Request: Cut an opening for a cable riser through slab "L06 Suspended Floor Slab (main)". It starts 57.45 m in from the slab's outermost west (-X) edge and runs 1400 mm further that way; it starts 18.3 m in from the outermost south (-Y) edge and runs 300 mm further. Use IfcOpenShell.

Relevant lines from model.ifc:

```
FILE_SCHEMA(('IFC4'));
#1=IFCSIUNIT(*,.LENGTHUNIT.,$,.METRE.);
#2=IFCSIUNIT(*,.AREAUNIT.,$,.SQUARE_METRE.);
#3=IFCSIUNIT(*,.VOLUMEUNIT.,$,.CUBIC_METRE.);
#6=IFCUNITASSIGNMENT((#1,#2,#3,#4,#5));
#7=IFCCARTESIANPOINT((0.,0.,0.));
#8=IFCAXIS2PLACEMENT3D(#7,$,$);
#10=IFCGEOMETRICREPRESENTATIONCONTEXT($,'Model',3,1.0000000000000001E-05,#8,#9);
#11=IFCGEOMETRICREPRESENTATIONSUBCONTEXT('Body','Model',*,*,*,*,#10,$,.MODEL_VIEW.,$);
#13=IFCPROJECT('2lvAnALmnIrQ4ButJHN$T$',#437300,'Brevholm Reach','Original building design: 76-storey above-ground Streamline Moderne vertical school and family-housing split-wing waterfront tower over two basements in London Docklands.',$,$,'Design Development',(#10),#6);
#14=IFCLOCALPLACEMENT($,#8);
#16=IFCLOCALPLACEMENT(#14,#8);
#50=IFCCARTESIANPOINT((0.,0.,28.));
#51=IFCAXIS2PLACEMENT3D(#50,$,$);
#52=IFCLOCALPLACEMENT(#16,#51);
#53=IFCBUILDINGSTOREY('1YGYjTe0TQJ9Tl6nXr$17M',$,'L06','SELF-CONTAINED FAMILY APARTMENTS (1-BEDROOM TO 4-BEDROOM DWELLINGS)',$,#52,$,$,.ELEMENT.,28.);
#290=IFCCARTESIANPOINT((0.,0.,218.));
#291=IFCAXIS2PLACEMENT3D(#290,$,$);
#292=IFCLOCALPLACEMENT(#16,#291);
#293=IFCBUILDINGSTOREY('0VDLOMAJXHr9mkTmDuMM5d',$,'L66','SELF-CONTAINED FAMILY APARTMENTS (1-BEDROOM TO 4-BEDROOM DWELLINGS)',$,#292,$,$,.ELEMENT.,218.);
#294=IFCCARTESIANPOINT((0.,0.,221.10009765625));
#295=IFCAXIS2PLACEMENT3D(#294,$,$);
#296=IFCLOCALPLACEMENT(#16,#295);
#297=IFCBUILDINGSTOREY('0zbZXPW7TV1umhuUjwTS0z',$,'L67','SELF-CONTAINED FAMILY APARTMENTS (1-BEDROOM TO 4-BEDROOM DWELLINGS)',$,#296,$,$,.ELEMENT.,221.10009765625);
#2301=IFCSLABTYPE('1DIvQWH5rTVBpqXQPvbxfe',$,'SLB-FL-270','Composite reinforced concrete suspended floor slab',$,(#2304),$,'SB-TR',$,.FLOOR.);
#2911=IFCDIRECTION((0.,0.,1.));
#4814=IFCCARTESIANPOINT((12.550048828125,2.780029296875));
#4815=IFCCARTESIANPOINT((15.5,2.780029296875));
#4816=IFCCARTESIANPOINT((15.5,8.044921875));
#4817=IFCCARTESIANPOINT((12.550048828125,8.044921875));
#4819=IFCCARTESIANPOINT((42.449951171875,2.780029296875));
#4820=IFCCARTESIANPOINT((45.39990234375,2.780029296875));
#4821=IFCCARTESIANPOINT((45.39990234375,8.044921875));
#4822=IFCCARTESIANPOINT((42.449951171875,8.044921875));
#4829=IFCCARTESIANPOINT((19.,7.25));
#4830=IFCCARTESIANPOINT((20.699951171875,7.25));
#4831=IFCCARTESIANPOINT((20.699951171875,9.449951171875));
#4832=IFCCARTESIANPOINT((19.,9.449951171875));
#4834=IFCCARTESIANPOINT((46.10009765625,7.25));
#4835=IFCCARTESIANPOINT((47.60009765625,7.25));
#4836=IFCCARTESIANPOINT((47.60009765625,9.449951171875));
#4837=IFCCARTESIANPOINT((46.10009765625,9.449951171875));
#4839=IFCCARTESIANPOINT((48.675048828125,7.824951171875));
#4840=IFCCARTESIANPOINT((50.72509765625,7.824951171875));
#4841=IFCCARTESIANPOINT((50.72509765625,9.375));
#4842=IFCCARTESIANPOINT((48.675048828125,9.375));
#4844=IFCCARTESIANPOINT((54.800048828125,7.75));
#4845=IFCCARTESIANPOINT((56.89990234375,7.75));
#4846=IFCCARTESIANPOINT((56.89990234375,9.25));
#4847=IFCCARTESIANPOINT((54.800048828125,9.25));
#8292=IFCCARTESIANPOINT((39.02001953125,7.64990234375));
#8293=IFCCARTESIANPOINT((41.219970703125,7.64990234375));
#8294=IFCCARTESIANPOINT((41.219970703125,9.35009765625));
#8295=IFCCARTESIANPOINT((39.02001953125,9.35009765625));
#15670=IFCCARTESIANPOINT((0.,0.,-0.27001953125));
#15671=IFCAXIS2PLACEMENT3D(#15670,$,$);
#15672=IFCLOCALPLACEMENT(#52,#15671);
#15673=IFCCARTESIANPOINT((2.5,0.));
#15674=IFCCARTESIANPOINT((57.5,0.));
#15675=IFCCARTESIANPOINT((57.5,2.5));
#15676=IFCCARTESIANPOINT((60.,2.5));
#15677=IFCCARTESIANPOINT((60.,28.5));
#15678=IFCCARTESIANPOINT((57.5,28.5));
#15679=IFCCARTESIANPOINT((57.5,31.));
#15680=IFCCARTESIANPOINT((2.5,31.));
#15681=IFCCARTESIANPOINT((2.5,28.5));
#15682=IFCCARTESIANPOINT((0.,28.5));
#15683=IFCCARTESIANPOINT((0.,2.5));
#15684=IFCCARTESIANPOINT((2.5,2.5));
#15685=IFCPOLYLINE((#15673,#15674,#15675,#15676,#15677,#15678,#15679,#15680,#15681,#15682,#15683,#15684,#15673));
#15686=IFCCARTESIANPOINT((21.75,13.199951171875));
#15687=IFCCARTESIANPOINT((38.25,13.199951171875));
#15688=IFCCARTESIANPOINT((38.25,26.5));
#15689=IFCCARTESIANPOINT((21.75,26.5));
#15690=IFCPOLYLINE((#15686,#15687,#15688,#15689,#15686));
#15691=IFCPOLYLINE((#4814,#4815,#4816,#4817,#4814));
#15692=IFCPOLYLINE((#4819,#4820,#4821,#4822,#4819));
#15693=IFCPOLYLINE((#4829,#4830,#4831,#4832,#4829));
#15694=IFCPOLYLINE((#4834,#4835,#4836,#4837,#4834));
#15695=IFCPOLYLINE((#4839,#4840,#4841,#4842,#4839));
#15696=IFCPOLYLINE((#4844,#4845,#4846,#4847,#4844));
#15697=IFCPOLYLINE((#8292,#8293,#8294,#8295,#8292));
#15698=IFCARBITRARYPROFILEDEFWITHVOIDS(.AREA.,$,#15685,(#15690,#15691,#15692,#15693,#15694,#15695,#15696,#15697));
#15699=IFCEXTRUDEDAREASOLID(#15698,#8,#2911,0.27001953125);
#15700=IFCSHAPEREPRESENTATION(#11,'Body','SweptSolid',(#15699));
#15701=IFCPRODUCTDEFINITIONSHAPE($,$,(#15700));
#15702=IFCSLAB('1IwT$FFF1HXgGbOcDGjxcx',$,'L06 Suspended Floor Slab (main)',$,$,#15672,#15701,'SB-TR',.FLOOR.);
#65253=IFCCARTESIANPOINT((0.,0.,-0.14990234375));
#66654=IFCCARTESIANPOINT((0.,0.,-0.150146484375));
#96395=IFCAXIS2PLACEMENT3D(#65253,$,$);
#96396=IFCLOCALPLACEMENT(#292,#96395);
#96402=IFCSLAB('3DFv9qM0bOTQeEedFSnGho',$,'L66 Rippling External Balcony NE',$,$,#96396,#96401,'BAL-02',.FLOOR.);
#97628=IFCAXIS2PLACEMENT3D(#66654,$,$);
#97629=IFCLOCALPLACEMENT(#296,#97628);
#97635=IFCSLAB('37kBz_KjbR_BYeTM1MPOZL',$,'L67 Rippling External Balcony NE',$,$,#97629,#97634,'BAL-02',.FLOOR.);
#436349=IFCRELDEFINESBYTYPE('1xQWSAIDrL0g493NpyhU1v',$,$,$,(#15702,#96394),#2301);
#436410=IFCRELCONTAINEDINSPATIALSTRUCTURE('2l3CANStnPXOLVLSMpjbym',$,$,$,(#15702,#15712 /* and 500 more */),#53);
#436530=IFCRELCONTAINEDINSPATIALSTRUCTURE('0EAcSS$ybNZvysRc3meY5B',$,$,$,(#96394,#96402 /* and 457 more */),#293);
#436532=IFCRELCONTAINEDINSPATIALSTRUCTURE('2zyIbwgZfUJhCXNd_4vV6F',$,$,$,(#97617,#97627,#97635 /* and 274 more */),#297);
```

```python
import numpy as np
import ifcopenshell
import ifcopenshell.api.feature
import ifcopenshell.api.geometry
import ifcopenshell.api.root
import ifcopenshell.geom
import ifcopenshell.util.placement
import ifcopenshell.util.representation
import ifcopenshell.util.shape
import ifcopenshell.util.unit

model = ifcopenshell.open("model.ifc")
unit_scale = ifcopenshell.util.unit.calculate_unit_scale(model)
settings = ifcopenshell.geom.settings()


def volume(element):
    """Net volume in cubic metres, openings subtracted."""
    shape = ifcopenshell.geom.create_shape(settings, element)
    return ifcopenshell.util.shape.get_volume(shape.geometry)


slab = model.by_guid("1IwT$FFF1HXgGbOcDGjxcx")
before = volume(slab)

# Extent in the slab's own axes, in metres. The edges named are its -X and -Y sides.
slab_shape = ifcopenshell.geom.create_shape(settings, slab)
vertices = ifcopenshell.util.shape.get_vertices(slab_shape.geometry)
x_min, y_min, bottom = vertices.min(axis=0)
top = vertices[:, 2].max()

opening = ifcopenshell.api.root.create_entity(model, ifc_class="IfcOpeningElement", name="Cable riser opening", predefined_type="OPENING")
context = ifcopenshell.util.representation.get_context(model, "Model", "Body", "MODEL_VIEW")
width, depth = 1.4, 0.3
outline = [(0.0, 0.0), (width, 0.0), (width, depth), (0.0, depth), (0.0, 0.0)]
# Overshoot both faces by 50 mm so the cut is clean.
shape = ifcopenshell.api.geometry.add_slab_representation(
    model, context=context, depth=top - bottom + 0.1, polyline=outline
)
ifcopenshell.api.geometry.assign_representation(model, product=opening, representation=shape)

matrix = ifcopenshell.util.placement.get_local_placement(slab.ObjectPlacement)
matrix[:, 3] = matrix @ np.append(np.array([x_min + 57.45, y_min + 18.3, bottom - 0.05]) / unit_scale, 1.0)
ifcopenshell.api.geometry.edit_object_placement(model, product=opening, matrix=matrix, is_si=False)
ifcopenshell.api.feature.add_feature(model, feature=opening, element=slab)

after = volume(slab)

print(f"slab volume {before:.3f} -> {after:.3f} m3")

model.write("model_updated.ifc")
```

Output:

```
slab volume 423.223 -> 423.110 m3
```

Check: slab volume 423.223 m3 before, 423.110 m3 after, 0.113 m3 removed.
